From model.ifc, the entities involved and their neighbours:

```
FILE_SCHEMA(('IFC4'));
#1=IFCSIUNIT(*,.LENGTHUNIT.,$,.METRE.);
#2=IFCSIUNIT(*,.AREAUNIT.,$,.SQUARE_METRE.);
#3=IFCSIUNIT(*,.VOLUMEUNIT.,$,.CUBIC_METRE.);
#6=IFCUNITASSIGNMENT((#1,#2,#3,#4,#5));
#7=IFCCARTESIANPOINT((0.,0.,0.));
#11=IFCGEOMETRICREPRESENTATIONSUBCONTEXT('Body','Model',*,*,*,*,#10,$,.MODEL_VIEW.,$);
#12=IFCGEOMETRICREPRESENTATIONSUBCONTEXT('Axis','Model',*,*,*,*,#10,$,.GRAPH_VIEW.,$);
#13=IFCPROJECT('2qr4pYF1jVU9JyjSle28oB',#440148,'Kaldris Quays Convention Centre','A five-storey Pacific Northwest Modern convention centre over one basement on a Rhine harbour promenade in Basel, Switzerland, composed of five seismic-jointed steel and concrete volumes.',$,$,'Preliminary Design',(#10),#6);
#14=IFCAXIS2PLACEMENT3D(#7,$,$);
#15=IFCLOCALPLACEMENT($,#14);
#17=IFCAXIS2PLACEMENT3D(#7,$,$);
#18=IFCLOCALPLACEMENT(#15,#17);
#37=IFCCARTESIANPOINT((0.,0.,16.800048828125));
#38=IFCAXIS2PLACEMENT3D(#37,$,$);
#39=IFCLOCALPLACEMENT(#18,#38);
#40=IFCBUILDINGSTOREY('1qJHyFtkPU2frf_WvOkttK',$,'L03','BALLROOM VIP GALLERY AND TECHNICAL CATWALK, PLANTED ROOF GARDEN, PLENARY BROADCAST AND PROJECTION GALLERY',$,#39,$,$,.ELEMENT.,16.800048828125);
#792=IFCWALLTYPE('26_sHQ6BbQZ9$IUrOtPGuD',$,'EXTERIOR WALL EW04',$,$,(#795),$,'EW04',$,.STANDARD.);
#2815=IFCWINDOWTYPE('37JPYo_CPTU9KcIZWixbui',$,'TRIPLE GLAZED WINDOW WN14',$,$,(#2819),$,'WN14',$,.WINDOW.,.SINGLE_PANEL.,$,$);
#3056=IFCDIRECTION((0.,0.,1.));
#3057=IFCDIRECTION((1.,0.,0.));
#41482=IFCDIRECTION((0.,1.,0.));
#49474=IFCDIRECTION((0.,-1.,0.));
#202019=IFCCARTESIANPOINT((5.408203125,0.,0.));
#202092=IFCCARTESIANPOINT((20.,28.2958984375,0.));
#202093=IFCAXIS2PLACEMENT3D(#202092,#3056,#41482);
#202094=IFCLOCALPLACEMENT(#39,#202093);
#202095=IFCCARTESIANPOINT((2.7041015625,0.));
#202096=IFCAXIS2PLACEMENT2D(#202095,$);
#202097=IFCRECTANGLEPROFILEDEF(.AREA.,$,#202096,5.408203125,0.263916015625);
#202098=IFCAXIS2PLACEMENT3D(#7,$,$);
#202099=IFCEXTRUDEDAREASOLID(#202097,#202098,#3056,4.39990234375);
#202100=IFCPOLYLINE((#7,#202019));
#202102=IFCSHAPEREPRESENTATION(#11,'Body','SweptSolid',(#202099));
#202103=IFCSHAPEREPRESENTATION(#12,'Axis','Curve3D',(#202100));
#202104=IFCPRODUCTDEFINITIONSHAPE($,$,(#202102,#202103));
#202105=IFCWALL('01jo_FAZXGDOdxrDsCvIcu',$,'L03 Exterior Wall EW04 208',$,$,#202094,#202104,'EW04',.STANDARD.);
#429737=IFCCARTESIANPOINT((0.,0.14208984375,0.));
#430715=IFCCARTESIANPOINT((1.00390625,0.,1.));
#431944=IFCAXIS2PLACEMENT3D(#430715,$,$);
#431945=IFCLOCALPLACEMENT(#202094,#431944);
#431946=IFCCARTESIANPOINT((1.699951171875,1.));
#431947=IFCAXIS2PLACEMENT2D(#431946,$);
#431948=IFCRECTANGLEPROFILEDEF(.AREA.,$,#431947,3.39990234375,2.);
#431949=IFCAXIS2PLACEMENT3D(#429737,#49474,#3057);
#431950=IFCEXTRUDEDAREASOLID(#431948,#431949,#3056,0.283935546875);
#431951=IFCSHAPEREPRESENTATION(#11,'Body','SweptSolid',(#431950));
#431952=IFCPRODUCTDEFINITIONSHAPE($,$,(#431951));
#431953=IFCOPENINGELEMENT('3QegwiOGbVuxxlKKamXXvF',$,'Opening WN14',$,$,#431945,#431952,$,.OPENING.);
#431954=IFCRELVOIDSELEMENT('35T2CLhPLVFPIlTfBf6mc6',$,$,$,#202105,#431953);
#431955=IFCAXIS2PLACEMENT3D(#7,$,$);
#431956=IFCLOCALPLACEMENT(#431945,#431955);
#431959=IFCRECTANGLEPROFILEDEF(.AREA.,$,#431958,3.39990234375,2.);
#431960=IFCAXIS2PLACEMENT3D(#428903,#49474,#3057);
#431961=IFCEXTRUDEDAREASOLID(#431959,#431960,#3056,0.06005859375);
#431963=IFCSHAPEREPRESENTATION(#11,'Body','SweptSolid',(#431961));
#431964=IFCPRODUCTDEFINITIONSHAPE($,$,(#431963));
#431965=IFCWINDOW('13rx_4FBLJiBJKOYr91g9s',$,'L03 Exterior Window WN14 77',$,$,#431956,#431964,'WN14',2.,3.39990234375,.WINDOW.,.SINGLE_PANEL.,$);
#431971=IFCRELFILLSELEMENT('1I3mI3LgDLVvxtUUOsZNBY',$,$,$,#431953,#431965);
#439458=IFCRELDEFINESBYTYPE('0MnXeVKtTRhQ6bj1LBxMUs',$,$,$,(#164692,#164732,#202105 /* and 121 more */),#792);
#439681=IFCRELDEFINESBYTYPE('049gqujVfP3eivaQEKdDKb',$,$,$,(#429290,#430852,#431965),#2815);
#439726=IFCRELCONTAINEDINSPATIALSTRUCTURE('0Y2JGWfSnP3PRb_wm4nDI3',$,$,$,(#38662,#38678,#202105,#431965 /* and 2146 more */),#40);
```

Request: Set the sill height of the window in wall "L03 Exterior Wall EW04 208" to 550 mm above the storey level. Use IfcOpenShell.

```python
import numpy as np
import ifcopenshell
import ifcopenshell.api.geometry
import ifcopenshell.geom
import ifcopenshell.util.element
import ifcopenshell.util.placement
import ifcopenshell.util.shape
import ifcopenshell.util.unit

model = ifcopenshell.open("model.ifc")
unit_scale = ifcopenshell.util.unit.calculate_unit_scale(model)

window = model.by_id(431965)
opening = window.FillsVoids[0].RelatingOpeningElement
storey = ifcopenshell.util.element.get_container(window, ifc_class="IfcBuildingStorey")
level = ifcopenshell.util.placement.get_local_placement(storey.ObjectPlacement)[2, 3]

# The opening's origin need not be at the sill, so measure its lowest point.
shape = ifcopenshell.geom.create_shape(ifcopenshell.geom.settings(), opening)
bottom = ifcopenshell.util.shape.get_shape_bottom_elevation(shape, shape.geometry) / unit_scale
dz = level + 0.55 - bottom

shift = np.array([0.0, 0.0, dz])
# The window is placed relative to its opening, so it follows when the opening moves.
matrix = ifcopenshell.util.placement.get_local_placement(opening.ObjectPlacement)
matrix[:3, 3] += shift
ifcopenshell.api.geometry.edit_object_placement(
    model, product=opening, matrix=matrix, is_si=False, should_transform_children=True
)

print(f"moved by {dz * unit_scale:+.3f} m")

model.write("model_v2.ifc")
```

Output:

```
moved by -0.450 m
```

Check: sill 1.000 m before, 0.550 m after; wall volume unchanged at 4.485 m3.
